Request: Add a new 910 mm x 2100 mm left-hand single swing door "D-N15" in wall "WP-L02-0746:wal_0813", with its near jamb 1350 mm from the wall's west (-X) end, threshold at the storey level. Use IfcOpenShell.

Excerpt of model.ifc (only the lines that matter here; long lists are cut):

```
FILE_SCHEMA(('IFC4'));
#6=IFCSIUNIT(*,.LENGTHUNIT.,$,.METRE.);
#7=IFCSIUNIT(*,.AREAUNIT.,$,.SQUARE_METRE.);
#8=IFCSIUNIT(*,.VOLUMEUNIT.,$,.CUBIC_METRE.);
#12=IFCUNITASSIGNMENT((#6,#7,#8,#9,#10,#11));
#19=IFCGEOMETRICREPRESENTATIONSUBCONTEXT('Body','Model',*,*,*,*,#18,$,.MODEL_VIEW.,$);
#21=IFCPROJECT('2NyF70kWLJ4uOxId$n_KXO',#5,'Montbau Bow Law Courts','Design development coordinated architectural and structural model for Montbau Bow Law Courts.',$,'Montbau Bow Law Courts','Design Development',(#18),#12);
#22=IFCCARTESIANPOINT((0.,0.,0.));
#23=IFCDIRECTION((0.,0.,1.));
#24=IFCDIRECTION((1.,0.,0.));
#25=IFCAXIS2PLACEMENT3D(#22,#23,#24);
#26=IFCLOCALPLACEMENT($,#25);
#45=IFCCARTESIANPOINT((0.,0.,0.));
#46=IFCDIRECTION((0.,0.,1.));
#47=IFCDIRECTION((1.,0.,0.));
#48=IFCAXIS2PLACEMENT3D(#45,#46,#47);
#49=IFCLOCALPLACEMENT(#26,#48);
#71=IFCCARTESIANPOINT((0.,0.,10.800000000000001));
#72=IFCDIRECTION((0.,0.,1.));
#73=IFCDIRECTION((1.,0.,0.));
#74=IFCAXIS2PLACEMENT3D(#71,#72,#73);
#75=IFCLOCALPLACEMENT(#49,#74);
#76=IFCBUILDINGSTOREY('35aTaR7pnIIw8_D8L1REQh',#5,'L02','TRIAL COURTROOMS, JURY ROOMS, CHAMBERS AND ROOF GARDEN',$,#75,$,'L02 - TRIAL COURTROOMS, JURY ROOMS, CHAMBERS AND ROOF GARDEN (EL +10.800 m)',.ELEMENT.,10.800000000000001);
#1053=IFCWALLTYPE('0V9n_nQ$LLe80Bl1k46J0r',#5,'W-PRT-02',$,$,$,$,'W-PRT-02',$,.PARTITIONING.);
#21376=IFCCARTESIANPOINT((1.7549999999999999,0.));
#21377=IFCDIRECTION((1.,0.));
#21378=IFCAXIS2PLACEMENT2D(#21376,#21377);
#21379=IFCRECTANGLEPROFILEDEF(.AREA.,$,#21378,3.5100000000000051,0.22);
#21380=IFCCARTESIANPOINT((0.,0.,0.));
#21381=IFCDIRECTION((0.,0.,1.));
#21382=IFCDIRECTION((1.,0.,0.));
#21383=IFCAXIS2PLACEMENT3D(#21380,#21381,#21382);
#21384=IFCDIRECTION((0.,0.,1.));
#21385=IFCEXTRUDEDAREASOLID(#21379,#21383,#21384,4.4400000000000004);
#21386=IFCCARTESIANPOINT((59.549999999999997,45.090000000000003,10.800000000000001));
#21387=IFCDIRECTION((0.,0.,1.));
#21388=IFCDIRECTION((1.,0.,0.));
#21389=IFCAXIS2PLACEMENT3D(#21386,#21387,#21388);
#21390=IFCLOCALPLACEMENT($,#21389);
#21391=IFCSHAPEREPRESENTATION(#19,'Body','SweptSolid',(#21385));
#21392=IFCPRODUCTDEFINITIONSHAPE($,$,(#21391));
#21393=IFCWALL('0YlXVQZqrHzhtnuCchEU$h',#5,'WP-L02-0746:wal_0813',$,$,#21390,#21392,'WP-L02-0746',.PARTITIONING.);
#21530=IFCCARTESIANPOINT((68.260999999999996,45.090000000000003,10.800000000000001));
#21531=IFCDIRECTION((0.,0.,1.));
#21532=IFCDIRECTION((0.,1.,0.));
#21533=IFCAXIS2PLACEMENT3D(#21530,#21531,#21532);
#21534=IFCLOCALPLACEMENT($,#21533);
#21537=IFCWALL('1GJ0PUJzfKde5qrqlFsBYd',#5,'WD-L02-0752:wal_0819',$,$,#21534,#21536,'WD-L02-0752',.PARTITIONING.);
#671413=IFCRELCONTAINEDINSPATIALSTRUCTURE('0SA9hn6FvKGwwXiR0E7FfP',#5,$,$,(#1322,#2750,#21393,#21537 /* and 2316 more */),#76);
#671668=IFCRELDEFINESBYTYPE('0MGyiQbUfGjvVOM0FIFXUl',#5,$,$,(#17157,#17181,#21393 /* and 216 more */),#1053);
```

```python
import numpy as np
import ifcopenshell
import ifcopenshell.api.feature
import ifcopenshell.api.geometry
import ifcopenshell.api.root
import ifcopenshell.api.spatial
import ifcopenshell.geom
import ifcopenshell.util.element
import ifcopenshell.util.placement
import ifcopenshell.util.representation
import ifcopenshell.util.shape
import ifcopenshell.util.unit

model = ifcopenshell.open("model.ifc")
unit_scale = ifcopenshell.util.unit.calculate_unit_scale(model)
settings = ifcopenshell.geom.settings()


def volume(element):
    """Net volume in cubic metres, openings subtracted."""
    shape = ifcopenshell.geom.create_shape(settings, element)
    return ifcopenshell.util.shape.get_volume(shape.geometry)


wall = model.by_guid("0YlXVQZqrHzhtnuCchEU$h")
storey = ifcopenshell.util.element.get_container(wall, ifc_class="IfcBuildingStorey")
context = ifcopenshell.util.representation.get_context(model, "Model", "Body", "MODEL_VIEW")
before = volume(wall)

width, height, from_end, sill = 0.91, 2.1, 1.35, 0.0  # metres

# The wall runs along its own X axis, and the end named is its -X end.
wall_shape = ifcopenshell.geom.create_shape(settings, wall)
x, y, z = ifcopenshell.util.shape.get_vertices(wall_shape.geometry).T
start = x.min() + from_end
face, thickness = float(y.min()), float(y.max() - y.min())
wall_matrix = ifcopenshell.util.placement.get_local_placement(wall.ObjectPlacement)
level = ifcopenshell.util.placement.get_local_placement(storey.ObjectPlacement)[2, 3]


def in_wall(x, y):
    """Placement at x, y metres in the wall's axes, at sill height."""
    matrix = wall_matrix.copy()
    matrix[:, 3] = wall_matrix @ np.array([x / unit_scale, y / unit_scale, 0.0, 1.0])
    matrix[2, 3] = level + sill / unit_scale
    return matrix


# Opening: a box that overshoots both wall faces by 50 mm.
opening = ifcopenshell.api.root.create_entity(model, ifc_class="IfcOpeningElement", predefined_type="OPENING")
box = ifcopenshell.api.geometry.add_wall_representation(
    model, context=context, length=width, height=height, thickness=thickness + 0.1
)
ifcopenshell.api.geometry.assign_representation(model, product=opening, representation=box)
ifcopenshell.api.geometry.edit_object_placement(model, product=opening, matrix=in_wall(start, face - 0.05), is_si=False)
ifcopenshell.api.feature.add_feature(model, feature=opening, element=wall)

door = ifcopenshell.api.root.create_entity(model, ifc_class="IfcDoor", name="D-N15", predefined_type="DOOR")
door.OverallWidth, door.OverallHeight = width / unit_scale, height / unit_scale
door.OperationType = "SINGLE_SWING_LEFT"
body = ifcopenshell.api.geometry.add_door_representation(
    model,
    context=context,
    overall_width=door.OverallWidth,
    overall_height=door.OverallHeight,
    operation_type="SINGLE_SWING_LEFT",
    lining_properties={"LiningDepth": thickness / unit_scale, "ThresholdDepth": thickness / unit_scale},
)
ifcopenshell.api.geometry.assign_representation(model, product=door, representation=body)
ifcopenshell.api.spatial.assign_container(model, products=[door], relating_structure=storey)
ifcopenshell.api.feature.add_filling(model, opening=opening, element=door)

# The lining spans the wall, so the door starts at the wall face.
ifcopenshell.api.geometry.edit_object_placement(model, product=door, matrix=in_wall(start, face), is_si=False)

after = volume(wall)

print(f"wall volume {before:.3f} -> {after:.3f} m3")

model.write("model_updated.ifc")
```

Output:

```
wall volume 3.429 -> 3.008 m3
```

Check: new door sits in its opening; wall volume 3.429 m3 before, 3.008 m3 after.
